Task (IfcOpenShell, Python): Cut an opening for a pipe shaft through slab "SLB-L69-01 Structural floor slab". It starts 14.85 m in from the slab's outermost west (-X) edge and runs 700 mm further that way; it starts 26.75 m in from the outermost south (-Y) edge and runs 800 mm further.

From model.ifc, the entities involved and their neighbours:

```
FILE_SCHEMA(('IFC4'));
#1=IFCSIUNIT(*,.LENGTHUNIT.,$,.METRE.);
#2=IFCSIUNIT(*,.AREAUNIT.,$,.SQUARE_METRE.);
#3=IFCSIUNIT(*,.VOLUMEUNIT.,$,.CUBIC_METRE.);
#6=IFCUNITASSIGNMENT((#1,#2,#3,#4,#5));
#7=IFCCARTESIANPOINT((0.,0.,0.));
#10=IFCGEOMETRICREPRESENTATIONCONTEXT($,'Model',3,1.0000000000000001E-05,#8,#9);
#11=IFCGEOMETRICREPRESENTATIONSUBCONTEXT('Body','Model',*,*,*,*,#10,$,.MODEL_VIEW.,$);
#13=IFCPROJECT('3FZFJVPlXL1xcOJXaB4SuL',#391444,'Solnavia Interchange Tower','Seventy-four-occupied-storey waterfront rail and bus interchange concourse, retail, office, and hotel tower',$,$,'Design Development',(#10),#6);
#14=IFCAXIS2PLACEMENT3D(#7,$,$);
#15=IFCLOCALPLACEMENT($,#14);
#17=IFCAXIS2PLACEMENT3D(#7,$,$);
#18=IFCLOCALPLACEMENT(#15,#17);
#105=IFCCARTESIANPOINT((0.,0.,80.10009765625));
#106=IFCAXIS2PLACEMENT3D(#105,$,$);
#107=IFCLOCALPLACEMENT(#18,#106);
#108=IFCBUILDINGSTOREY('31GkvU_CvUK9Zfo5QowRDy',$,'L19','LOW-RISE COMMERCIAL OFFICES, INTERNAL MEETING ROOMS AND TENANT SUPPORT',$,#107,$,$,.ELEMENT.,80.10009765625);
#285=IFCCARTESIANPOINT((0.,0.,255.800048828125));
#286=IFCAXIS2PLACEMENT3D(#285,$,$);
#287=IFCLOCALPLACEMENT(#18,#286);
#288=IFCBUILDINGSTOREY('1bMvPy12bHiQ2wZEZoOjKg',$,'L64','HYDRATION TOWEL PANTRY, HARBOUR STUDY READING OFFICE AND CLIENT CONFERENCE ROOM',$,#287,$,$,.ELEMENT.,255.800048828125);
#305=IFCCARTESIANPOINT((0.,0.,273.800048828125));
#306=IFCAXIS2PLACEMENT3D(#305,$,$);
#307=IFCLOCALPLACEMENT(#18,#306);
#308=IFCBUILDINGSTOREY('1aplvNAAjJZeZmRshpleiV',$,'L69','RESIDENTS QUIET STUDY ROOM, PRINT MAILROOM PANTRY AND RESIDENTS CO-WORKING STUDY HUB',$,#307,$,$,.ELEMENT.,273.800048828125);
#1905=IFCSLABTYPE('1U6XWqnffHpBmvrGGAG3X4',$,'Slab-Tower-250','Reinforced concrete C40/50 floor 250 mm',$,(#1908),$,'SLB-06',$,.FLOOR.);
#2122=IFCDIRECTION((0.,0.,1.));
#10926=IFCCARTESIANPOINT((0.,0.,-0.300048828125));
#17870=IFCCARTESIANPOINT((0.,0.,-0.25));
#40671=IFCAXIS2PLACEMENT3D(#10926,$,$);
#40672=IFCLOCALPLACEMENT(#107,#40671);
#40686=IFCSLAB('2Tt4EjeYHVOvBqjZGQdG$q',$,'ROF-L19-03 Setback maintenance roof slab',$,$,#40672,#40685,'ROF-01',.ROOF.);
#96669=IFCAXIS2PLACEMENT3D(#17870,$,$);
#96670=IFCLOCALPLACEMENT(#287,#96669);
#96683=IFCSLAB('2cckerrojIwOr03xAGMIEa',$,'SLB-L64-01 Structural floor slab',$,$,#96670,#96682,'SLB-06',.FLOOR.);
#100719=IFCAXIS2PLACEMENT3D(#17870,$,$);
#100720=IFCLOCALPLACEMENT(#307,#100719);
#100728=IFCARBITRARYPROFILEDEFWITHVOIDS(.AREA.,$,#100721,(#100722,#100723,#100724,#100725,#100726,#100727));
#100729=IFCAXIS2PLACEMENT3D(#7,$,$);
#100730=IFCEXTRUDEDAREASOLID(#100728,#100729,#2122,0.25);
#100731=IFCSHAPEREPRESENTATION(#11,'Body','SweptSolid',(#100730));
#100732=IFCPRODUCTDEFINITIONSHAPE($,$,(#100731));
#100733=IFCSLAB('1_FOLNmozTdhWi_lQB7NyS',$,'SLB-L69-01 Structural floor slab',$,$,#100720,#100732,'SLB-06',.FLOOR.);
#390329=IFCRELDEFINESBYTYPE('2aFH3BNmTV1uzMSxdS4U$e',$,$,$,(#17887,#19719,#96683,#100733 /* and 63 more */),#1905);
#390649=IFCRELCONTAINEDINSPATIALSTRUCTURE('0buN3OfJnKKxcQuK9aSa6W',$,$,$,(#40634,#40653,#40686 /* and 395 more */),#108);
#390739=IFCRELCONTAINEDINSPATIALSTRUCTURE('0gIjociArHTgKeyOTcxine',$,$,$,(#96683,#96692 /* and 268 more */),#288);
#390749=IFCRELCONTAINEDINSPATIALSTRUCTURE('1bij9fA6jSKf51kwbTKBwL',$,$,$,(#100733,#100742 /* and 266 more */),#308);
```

```python
import numpy as np
import ifcopenshell
import ifcopenshell.api.feature
import ifcopenshell.api.geometry
import ifcopenshell.api.root
import ifcopenshell.geom
import ifcopenshell.util.placement
import ifcopenshell.util.representation
import ifcopenshell.util.shape
import ifcopenshell.util.unit

model = ifcopenshell.open("model.ifc")
unit_scale = ifcopenshell.util.unit.calculate_unit_scale(model)
settings = ifcopenshell.geom.settings()


def volume(element):
    """Net volume in cubic metres, openings subtracted."""
    shape = ifcopenshell.geom.create_shape(settings, element)
    return ifcopenshell.util.shape.get_volume(shape.geometry)


slab = model.by_id(100733)
before = volume(slab)

# Extent in the slab's own axes, in metres. The edges named are its -X and -Y sides.
slab_shape = ifcopenshell.geom.create_shape(settings, slab)
vertices = ifcopenshell.util.shape.get_vertices(slab_shape.geometry)
x_min, y_min, bottom = vertices.min(axis=0)
top = vertices[:, 2].max()

opening = ifcopenshell.api.root.create_entity(model, ifc_class="IfcOpeningElement", name="Pipe shaft opening", predefined_type="OPENING")
context = ifcopenshell.util.representation.get_context(model, "Model", "Body", "MODEL_VIEW")
width, depth = 0.7, 0.8
outline = [(0.0, 0.0), (width, 0.0), (width, depth), (0.0, depth), (0.0, 0.0)]
# Overshoot both faces by 50 mm so the cut is clean.
shape = ifcopenshell.api.geometry.add_slab_representation(
    model, context=context, depth=top - bottom + 0.1, polyline=outline
)
ifcopenshell.api.geometry.assign_representation(model, product=opening, representation=shape)

matrix = ifcopenshell.util.placement.get_local_placement(slab.ObjectPlacement)
matrix[:, 3] = matrix @ np.append(np.array([x_min + 14.85, y_min + 26.75, bottom - 0.05]) / unit_scale, 1.0)
ifcopenshell.api.geometry.edit_object_placement(model, product=opening, matrix=matrix, is_si=False)
ifcopenshell.api.feature.add_feature(model, feature=opening, element=slab)

after = volume(slab)

print(f"slab volume {before:.3f} -> {after:.3f} m3")

model.write("model-out.ifc")
```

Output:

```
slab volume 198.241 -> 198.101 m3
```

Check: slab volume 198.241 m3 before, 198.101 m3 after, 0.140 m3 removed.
